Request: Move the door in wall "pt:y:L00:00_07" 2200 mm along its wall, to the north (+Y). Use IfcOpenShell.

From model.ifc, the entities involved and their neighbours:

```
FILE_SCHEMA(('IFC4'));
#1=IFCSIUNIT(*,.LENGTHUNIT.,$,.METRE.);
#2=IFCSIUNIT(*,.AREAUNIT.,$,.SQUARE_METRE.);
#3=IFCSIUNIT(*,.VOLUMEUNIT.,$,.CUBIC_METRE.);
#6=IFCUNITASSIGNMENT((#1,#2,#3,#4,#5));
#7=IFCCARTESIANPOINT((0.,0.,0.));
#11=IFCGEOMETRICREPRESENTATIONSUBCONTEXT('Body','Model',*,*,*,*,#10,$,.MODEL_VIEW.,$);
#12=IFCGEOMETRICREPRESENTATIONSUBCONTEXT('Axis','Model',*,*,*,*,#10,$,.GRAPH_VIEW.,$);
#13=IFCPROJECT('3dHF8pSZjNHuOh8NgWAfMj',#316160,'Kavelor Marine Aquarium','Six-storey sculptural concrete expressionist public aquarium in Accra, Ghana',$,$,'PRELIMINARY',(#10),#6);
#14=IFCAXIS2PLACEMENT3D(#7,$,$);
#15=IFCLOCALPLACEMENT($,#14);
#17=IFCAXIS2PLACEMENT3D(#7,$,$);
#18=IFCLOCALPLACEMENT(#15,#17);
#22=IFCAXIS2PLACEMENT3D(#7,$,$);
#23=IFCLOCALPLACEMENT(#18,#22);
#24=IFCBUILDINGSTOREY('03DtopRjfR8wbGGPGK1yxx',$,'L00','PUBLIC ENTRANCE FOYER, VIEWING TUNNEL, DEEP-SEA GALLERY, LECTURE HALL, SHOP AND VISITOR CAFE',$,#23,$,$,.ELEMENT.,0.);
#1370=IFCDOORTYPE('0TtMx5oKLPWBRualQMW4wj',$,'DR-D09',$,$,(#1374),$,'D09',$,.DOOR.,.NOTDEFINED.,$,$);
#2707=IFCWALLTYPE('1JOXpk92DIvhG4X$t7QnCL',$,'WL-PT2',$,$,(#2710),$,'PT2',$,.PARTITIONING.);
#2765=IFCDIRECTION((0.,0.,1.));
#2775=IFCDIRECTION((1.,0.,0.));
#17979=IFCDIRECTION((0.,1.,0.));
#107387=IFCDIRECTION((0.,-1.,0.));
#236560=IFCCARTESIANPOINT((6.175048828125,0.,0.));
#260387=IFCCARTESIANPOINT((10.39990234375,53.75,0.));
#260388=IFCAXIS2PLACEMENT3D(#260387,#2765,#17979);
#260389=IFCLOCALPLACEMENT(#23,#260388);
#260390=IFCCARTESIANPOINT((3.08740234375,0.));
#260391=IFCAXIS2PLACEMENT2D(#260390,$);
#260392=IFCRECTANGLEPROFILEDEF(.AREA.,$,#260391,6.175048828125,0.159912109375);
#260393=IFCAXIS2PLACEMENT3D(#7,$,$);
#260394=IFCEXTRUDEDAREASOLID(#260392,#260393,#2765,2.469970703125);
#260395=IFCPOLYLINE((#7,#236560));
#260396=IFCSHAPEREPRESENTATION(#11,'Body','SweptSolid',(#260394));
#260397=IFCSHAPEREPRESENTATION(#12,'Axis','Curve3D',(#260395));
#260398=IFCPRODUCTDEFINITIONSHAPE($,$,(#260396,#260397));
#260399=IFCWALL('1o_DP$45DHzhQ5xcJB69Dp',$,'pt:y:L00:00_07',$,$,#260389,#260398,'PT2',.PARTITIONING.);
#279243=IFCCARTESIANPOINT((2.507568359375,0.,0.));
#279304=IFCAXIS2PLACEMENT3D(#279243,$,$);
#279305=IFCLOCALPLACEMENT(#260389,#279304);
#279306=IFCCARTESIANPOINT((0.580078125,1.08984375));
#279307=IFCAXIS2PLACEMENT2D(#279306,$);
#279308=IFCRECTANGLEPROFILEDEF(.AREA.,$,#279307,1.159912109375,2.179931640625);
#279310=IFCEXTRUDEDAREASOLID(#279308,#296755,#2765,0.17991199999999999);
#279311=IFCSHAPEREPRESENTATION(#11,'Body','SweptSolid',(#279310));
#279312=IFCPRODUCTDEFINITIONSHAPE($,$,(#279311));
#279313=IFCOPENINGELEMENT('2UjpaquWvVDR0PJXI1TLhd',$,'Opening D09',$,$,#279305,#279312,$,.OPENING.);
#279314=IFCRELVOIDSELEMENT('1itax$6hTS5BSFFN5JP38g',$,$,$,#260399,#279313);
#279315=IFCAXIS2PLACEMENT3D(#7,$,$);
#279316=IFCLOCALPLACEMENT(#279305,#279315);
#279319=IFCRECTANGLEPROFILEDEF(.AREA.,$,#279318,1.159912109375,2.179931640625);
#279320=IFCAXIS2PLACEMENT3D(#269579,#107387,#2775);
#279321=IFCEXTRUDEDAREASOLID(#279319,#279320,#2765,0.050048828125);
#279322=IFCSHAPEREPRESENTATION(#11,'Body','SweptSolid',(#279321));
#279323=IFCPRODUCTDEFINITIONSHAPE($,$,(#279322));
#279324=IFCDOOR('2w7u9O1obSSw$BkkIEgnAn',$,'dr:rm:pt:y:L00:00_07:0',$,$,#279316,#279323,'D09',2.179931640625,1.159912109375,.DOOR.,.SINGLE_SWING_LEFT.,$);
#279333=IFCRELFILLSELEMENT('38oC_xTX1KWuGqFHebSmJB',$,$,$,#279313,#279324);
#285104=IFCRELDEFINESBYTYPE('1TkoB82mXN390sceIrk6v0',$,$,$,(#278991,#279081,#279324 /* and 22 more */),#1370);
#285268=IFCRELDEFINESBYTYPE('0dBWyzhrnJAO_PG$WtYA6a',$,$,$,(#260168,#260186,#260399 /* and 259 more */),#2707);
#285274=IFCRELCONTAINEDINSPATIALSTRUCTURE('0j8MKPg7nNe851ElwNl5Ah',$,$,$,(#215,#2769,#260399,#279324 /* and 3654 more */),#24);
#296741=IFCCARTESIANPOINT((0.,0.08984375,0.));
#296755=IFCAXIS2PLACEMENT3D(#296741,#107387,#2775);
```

```python
import ifcopenshell
import ifcopenshell.api.geometry
import ifcopenshell.util.placement
import ifcopenshell.util.unit

model = ifcopenshell.open("model.ifc")
unit_scale = ifcopenshell.util.unit.calculate_unit_scale(model)

door = model.by_guid("2w7u9O1obSSw$BkkIEgnAn")
opening = door.FillsVoids[0].RelatingOpeningElement
wall = opening.VoidsElements[0].RelatingBuildingElement

wall_matrix = ifcopenshell.util.placement.get_local_placement(wall.ObjectPlacement)
shift = wall_matrix[:3, 0] * 2.2 / unit_scale
before = ifcopenshell.util.placement.get_local_placement(door.ObjectPlacement)[:3, 3].copy()

# The door is placed relative to its opening, so it follows when the opening moves.
matrix = ifcopenshell.util.placement.get_local_placement(opening.ObjectPlacement)
matrix[:3, 3] += shift
ifcopenshell.api.geometry.edit_object_placement(
    model, product=opening, matrix=matrix, is_si=False, should_transform_children=True
)

after = ifcopenshell.util.placement.get_local_placement(door.ObjectPlacement)[:3, 3]
print("door moved by", (after - before).round(3) + 0.0)

model.write("model-out.ifc")
```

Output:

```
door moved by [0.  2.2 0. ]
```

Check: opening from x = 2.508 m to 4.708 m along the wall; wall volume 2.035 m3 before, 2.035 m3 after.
